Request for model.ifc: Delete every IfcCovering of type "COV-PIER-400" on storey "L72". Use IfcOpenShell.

First a look at what the model holds.

```python
import ifcopenshell
import ifcopenshell.util.element

model = ifcopenshell.open("model.ifc")
print(model.schema)
storey = next(s for s in model.by_type("IfcBuildingStorey") if s.Name == "L72")
coverings = [e for e in ifcopenshell.util.element.get_decomposition(storey) if e.is_a("IfcCovering")]
seen = {}
for e in coverings:
    element_type = ifcopenshell.util.element.get_type(e)
    name = element_type.Name if element_type not in (None, e) else None
    seen[name] = seen.get(name, 0) + 1
for name, count in sorted(seen.items(), key=str):
    print(count, "x", name)
```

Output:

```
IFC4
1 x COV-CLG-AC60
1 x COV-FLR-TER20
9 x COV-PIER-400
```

```python
import ifcopenshell
import ifcopenshell.api.root
import ifcopenshell.util.element

model = ifcopenshell.open("model.ifc")

storey = next(s for s in model.by_type("IfcBuildingStorey") if s.Name == "L72")
coverings = [e for e in ifcopenshell.util.element.get_decomposition(storey) if e.is_a("IfcCovering")]
targets = [e for e in coverings if (t := ifcopenshell.util.element.get_type(e)) not in (None, e) and t.Name == "COV-PIER-400"]

for e in targets:
    ifcopenshell.api.root.remove_product(model, product=e)
print(len(targets), "removed")

model.write("model_updated.ifc")
```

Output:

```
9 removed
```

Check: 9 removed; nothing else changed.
